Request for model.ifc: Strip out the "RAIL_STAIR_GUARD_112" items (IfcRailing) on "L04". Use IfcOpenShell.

First a look at what the model holds.

```python
import ifcopenshell
import ifcopenshell.util.element

model = ifcopenshell.open("model.ifc")
print(model.schema)
storey = next(s for s in model.by_type("IfcBuildingStorey") if s.Name == "L04")
railings = [e for e in ifcopenshell.util.element.get_decomposition(storey) if e.is_a("IfcRailing")]
seen = {}
for e in railings:
    element_type = ifcopenshell.util.element.get_type(e)
    name = element_type.Name if element_type not in (None, e) else None
    seen[name] = seen.get(name, 0) + 1
for name, count in sorted(seen.items(), key=str):
    print(count, "x", name)
```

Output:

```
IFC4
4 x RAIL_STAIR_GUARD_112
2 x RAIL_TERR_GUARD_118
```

```python
import ifcopenshell
import ifcopenshell.api.root
import ifcopenshell.util.element

model = ifcopenshell.open("model.ifc")

storey = next(s for s in model.by_type("IfcBuildingStorey") if s.Name == "L04")
railings = [e for e in ifcopenshell.util.element.get_decomposition(storey) if e.is_a("IfcRailing")]
targets = [e for e in railings if (t := ifcopenshell.util.element.get_type(e)) not in (None, e) and t.Name == "RAIL_STAIR_GUARD_112"]

for e in targets:
    ifcopenshell.api.root.remove_product(model, product=e)
print(len(targets), "removed")

model.write("model-out.ifc")
```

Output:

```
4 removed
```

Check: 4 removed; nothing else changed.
